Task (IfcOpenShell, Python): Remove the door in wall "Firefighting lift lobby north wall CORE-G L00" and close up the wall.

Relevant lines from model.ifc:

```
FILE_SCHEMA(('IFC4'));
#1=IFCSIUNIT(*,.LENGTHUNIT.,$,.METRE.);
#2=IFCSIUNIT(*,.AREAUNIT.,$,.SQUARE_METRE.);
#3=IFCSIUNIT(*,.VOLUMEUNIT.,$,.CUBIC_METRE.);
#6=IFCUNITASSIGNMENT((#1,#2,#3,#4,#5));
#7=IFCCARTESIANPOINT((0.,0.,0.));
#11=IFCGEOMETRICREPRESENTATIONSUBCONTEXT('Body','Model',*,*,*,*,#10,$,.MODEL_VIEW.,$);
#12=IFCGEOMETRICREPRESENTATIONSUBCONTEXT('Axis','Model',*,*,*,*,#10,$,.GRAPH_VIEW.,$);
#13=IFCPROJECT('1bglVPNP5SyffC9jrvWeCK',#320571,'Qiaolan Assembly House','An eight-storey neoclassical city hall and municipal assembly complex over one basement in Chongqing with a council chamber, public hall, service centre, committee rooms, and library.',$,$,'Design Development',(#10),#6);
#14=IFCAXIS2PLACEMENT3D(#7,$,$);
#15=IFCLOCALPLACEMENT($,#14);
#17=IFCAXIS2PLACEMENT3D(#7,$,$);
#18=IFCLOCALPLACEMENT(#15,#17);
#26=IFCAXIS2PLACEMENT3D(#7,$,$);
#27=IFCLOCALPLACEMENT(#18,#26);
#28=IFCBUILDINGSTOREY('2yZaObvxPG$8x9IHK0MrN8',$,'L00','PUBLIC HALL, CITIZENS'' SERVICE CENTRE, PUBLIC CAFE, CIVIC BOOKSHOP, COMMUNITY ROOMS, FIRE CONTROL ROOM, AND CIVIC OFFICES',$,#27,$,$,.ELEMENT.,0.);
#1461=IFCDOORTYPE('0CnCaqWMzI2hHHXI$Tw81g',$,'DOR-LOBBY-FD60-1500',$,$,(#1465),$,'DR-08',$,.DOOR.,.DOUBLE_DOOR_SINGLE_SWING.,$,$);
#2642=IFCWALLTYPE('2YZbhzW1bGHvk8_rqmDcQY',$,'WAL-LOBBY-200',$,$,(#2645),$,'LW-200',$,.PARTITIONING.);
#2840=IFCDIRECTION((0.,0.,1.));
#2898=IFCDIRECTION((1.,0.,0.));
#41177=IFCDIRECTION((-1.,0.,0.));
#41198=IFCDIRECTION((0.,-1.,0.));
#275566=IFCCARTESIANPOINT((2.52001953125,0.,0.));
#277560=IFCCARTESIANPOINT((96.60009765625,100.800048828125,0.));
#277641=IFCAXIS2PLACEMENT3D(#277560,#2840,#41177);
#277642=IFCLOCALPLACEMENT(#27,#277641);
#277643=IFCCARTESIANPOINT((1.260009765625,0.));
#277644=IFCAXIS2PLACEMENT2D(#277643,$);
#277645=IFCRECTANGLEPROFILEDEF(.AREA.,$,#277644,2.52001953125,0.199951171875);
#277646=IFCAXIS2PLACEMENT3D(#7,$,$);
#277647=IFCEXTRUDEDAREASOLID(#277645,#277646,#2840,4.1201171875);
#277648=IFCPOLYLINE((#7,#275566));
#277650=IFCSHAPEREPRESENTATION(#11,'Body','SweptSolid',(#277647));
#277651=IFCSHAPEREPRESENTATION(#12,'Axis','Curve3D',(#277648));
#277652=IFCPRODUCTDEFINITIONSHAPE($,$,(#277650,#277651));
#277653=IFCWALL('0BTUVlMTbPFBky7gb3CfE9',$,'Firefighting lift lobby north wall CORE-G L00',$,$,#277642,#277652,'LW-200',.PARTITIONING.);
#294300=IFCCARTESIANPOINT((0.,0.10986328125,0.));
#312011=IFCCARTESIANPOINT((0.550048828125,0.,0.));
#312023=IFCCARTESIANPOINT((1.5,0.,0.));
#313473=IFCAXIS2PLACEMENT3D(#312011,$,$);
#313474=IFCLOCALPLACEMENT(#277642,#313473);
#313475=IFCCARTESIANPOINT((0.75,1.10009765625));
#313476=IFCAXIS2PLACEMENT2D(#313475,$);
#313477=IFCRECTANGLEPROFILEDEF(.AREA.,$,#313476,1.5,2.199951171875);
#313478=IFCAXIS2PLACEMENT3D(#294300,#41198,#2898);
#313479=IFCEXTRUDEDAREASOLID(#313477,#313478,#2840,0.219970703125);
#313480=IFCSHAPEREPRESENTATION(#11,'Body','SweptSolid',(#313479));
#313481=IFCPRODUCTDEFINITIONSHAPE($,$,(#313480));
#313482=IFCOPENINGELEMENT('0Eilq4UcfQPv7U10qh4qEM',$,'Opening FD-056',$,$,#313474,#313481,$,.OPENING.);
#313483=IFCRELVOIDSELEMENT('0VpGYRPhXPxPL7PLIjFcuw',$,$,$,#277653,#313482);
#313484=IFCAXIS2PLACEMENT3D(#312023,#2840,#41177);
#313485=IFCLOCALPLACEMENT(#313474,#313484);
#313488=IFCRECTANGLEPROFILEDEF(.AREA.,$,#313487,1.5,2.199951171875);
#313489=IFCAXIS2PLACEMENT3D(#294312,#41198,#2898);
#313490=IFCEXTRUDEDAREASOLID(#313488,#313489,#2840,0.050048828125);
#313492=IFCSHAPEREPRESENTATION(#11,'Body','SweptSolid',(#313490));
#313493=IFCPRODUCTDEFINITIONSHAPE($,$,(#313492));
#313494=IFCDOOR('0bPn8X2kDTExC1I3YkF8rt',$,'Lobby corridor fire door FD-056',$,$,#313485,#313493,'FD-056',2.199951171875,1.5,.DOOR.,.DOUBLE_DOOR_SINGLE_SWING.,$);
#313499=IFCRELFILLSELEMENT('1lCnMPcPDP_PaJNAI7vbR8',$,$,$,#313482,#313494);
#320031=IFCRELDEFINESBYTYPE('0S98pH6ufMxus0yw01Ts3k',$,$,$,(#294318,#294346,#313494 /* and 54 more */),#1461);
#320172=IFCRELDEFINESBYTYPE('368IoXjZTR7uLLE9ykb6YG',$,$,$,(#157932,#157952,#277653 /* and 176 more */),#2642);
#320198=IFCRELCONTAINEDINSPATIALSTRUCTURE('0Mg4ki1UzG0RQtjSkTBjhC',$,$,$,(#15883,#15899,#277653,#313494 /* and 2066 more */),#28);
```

```python
import ifcopenshell
import ifcopenshell.api.feature
import ifcopenshell.api.root
import ifcopenshell.geom
import ifcopenshell.util.shape

model = ifcopenshell.open("model.ifc")
settings = ifcopenshell.geom.settings()


def volume(element):
    """Net volume in cubic metres, openings subtracted."""
    shape = ifcopenshell.geom.create_shape(settings, element)
    return ifcopenshell.util.shape.get_volume(shape.geometry)


door = model.by_id(313494)
opening = door.FillsVoids[0].RelatingOpeningElement
wall = opening.VoidsElements[0].RelatingBuildingElement
before = volume(wall)

ifcopenshell.api.root.remove_product(model, product=door)
ifcopenshell.api.feature.remove_feature(model, feature=opening)

after = volume(wall)

print(f"wall volume {before:.3f} -> {after:.3f} m3")

model.write("model_updated.ifc")
```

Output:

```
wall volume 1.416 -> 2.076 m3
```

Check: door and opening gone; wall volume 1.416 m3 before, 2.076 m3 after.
